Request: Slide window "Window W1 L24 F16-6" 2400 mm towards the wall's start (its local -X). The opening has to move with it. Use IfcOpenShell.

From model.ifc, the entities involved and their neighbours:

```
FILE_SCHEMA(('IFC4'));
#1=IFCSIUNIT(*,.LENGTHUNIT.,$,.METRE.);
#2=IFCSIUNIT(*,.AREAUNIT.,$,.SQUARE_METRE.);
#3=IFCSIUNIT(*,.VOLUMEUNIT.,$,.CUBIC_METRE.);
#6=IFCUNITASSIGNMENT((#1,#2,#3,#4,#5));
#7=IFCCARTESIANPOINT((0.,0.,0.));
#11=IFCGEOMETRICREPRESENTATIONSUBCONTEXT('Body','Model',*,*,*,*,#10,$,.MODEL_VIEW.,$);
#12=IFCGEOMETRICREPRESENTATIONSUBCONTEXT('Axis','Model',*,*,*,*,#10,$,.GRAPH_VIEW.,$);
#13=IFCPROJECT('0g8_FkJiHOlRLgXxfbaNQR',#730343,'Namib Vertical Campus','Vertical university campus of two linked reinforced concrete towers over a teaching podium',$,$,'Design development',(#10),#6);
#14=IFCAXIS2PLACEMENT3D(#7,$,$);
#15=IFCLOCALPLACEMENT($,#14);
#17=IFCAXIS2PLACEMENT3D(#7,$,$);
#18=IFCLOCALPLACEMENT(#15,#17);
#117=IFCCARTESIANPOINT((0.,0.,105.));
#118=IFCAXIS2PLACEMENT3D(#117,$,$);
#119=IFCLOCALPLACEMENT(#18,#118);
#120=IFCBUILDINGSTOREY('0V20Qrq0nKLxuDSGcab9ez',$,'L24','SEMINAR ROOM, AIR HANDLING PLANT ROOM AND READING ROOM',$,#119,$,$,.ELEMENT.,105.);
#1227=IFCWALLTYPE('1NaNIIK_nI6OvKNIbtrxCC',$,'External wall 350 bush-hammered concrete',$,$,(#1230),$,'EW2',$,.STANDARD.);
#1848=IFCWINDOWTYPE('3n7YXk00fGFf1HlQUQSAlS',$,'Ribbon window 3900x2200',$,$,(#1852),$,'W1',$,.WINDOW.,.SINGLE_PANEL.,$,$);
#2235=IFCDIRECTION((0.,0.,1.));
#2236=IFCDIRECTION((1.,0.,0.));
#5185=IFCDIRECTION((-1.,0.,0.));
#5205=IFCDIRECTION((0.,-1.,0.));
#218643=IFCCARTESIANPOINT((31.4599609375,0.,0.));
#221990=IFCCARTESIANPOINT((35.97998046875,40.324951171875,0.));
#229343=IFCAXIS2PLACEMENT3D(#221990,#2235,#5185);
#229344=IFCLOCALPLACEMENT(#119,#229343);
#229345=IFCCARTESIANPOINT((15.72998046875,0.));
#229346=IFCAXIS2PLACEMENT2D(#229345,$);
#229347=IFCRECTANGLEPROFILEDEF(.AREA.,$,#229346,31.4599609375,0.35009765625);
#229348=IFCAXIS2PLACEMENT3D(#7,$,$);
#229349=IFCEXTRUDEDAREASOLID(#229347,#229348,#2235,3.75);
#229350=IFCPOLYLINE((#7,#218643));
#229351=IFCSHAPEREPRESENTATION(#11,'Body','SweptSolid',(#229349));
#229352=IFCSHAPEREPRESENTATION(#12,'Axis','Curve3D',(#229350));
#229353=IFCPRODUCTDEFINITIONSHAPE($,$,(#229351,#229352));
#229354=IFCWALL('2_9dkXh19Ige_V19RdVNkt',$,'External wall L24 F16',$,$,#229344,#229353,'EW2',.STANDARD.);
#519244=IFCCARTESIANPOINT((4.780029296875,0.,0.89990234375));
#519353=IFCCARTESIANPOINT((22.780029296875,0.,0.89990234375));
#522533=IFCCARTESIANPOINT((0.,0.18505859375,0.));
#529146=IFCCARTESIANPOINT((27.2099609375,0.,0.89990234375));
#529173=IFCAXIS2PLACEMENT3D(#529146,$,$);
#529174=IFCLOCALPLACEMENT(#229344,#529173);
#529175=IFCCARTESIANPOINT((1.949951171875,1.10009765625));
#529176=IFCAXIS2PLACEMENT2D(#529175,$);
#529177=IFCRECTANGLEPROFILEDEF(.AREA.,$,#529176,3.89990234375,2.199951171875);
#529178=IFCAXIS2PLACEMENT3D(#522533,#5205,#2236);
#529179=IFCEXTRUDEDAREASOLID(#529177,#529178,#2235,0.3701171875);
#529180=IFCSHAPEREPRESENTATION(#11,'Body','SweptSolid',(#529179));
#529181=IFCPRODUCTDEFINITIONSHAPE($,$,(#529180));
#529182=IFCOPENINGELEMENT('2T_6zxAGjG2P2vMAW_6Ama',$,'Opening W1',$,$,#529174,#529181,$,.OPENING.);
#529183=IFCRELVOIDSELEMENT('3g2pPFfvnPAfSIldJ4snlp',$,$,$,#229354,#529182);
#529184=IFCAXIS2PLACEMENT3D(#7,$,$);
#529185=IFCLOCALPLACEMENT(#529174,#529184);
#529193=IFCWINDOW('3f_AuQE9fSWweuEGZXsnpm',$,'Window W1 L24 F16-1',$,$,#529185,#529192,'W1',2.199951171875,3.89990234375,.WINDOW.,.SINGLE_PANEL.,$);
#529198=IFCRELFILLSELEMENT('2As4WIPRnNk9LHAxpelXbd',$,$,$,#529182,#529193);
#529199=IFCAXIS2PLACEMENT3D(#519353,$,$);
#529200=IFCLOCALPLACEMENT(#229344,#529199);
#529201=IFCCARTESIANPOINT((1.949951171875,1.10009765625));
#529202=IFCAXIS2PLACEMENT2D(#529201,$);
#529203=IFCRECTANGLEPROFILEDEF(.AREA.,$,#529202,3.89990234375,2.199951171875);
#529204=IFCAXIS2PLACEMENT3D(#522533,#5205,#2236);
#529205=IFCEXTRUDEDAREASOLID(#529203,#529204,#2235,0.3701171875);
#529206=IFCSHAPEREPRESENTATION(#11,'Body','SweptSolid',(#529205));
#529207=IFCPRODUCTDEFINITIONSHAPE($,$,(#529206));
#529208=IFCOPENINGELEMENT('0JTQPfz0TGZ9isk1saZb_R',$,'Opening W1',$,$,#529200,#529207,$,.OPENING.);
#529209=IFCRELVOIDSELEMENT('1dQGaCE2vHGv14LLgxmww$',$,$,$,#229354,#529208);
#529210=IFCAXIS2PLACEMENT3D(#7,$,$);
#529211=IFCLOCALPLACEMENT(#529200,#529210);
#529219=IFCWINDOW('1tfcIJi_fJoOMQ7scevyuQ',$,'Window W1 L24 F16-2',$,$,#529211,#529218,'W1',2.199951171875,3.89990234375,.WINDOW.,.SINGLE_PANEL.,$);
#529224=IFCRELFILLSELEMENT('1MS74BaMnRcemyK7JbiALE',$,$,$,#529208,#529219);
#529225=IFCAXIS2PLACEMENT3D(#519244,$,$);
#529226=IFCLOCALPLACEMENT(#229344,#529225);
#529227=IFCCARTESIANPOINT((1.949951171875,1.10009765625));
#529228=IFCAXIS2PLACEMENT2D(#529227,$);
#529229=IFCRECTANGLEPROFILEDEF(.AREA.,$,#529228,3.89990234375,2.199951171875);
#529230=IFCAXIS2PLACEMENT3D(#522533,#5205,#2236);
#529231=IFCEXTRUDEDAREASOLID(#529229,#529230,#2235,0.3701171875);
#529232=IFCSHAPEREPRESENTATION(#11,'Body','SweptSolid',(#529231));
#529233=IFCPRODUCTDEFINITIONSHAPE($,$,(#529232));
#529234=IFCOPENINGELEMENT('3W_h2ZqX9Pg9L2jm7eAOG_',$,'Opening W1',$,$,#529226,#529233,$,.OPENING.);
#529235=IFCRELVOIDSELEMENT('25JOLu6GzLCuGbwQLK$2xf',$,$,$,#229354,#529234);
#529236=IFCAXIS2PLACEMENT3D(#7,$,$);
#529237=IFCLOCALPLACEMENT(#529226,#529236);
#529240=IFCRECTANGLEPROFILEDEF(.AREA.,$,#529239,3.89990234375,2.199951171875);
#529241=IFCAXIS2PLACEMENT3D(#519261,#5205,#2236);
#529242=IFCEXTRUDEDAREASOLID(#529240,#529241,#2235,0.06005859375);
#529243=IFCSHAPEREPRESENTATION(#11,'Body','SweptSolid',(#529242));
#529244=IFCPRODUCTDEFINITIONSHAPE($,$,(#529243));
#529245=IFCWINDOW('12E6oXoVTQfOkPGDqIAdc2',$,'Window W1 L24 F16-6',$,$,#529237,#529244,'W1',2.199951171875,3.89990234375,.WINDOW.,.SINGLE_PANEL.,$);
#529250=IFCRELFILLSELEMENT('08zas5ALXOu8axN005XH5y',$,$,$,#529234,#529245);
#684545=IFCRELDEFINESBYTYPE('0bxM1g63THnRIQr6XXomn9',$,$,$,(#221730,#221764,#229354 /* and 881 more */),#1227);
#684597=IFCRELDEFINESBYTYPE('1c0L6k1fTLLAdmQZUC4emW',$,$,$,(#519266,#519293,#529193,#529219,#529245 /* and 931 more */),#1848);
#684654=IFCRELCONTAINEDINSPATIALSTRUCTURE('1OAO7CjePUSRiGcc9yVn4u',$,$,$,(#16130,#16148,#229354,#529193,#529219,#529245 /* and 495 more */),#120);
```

```python
import ifcopenshell
import ifcopenshell.api.geometry
import ifcopenshell.util.placement

model = ifcopenshell.open("model.ifc")

window = model.by_guid("12E6oXoVTQfOkPGDqIAdc2")
opening = window.FillsVoids[0].RelatingOpeningElement
wall = opening.VoidsElements[0].RelatingBuildingElement

wall_matrix = ifcopenshell.util.placement.get_local_placement(wall.ObjectPlacement)
shift = wall_matrix[:3, 0] * -2.4
before = ifcopenshell.util.placement.get_local_placement(window.ObjectPlacement)[:3, 3].copy()

# The window is placed relative to its opening, so it follows when the opening moves.
matrix = ifcopenshell.util.placement.get_local_placement(opening.ObjectPlacement)
matrix[:3, 3] += shift
ifcopenshell.api.geometry.edit_object_placement(
    model, product=opening, matrix=matrix, is_si=False, should_transform_children=True
)

after = ifcopenshell.util.placement.get_local_placement(window.ObjectPlacement)[:3, 3]
print("window moved by", (after - before).round(3) + 0.0)

model.write("model_v2.ifc")
```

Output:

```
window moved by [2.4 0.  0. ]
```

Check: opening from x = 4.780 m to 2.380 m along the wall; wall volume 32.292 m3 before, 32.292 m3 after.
